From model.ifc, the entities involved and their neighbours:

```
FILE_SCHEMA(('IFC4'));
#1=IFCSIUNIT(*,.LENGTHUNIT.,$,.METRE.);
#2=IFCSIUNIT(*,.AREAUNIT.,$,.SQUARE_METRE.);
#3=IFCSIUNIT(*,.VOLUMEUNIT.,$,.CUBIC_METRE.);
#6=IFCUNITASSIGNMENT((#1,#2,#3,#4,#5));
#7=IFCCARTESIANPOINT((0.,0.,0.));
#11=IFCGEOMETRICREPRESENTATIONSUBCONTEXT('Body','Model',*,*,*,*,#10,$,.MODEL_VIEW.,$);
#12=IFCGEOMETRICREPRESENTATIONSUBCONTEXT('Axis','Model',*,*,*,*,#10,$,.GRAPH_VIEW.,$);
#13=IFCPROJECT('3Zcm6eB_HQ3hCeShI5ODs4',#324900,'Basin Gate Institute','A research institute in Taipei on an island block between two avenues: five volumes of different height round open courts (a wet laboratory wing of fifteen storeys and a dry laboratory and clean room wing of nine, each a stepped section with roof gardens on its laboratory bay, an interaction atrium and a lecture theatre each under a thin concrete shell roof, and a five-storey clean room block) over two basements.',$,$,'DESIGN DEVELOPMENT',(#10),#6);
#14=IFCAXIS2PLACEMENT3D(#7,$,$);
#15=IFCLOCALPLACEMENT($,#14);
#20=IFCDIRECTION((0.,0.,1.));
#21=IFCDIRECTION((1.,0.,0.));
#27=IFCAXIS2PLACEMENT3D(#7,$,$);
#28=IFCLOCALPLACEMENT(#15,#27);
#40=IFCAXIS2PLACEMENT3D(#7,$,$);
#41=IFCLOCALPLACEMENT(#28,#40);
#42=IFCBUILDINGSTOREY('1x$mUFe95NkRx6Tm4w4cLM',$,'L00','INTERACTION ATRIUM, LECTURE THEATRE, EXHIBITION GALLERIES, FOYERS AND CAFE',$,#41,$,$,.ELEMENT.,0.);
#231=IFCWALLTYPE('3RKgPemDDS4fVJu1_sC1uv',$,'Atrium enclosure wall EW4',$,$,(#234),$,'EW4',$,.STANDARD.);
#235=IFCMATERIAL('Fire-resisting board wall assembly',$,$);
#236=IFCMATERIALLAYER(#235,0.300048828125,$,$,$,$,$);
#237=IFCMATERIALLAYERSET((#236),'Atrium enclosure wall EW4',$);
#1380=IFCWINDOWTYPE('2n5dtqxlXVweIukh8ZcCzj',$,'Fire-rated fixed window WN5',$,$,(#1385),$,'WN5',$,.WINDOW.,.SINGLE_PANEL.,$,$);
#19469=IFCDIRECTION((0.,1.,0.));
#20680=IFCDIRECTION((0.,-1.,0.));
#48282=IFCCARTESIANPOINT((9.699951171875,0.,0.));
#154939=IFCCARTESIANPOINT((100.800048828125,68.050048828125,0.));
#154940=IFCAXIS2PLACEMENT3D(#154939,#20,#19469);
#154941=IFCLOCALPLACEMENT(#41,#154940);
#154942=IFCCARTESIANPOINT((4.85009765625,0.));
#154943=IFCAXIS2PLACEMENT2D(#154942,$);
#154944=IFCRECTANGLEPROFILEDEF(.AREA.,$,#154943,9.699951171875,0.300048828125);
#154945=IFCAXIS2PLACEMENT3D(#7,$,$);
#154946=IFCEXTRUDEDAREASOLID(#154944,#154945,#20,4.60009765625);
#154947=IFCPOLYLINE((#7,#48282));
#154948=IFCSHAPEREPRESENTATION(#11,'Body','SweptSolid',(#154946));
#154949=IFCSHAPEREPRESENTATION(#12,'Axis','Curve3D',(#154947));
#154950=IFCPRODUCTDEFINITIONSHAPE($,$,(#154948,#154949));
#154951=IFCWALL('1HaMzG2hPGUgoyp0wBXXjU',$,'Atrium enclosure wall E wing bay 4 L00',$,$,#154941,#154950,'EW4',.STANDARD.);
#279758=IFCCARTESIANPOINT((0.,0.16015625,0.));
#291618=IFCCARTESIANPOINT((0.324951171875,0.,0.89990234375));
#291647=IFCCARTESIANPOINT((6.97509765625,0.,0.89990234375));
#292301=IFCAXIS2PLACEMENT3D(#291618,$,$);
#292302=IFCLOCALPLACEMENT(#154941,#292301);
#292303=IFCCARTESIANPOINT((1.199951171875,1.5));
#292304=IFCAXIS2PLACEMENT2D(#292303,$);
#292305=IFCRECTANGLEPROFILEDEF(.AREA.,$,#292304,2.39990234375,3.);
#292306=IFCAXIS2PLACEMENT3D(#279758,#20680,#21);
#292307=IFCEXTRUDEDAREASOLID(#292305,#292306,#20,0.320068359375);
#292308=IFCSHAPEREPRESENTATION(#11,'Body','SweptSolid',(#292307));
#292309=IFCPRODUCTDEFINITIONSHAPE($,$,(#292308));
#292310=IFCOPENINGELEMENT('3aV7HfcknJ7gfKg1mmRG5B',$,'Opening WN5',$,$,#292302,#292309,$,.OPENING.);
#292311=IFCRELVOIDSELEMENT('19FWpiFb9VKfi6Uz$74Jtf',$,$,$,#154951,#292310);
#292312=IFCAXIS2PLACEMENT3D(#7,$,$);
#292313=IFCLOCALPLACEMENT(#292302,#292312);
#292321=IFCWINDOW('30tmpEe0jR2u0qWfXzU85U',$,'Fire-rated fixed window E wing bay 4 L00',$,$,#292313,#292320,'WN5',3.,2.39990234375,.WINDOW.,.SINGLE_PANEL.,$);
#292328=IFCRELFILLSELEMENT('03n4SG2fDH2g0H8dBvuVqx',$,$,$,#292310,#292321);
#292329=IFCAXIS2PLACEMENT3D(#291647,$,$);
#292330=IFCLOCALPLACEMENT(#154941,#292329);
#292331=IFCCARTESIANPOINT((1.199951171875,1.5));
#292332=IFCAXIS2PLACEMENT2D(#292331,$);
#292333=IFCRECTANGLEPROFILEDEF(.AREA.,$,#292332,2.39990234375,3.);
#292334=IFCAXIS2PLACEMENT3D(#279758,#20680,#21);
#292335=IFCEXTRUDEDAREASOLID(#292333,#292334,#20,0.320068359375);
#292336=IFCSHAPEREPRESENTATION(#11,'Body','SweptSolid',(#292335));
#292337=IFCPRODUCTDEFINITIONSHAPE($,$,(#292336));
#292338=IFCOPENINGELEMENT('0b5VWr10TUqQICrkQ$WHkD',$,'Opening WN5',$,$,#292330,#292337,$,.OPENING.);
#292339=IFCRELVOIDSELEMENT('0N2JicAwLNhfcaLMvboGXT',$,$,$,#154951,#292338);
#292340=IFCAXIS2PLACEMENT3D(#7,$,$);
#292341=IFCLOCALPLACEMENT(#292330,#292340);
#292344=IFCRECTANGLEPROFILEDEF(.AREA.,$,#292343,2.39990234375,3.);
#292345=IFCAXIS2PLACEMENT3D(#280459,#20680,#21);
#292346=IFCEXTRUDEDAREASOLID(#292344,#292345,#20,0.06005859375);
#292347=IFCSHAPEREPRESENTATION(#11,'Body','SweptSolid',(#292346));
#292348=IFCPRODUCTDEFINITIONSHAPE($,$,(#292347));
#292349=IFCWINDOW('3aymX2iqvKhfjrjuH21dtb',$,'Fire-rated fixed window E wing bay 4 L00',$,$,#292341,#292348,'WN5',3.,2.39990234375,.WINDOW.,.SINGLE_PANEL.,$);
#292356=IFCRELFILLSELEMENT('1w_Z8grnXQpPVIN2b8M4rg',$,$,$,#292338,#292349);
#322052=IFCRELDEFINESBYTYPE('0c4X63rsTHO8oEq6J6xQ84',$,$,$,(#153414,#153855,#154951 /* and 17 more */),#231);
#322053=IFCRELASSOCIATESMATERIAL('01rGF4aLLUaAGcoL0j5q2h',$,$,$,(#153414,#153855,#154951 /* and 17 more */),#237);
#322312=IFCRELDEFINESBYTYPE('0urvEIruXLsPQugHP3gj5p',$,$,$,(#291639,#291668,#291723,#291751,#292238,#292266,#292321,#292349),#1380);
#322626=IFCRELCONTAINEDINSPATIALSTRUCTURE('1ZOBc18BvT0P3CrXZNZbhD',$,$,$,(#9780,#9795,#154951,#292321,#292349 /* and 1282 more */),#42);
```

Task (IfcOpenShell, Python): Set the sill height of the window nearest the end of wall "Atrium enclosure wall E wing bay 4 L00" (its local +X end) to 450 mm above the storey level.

```python
import numpy as np
import ifcopenshell
import ifcopenshell.api.geometry
import ifcopenshell.geom
import ifcopenshell.util.element
import ifcopenshell.util.placement
import ifcopenshell.util.shape
import ifcopenshell.util.unit

model = ifcopenshell.open("model.ifc")
unit_scale = ifcopenshell.util.unit.calculate_unit_scale(model)

window = model.by_id(292349)
opening = window.FillsVoids[0].RelatingOpeningElement
storey = ifcopenshell.util.element.get_container(window, ifc_class="IfcBuildingStorey")
level = ifcopenshell.util.placement.get_local_placement(storey.ObjectPlacement)[2, 3]

# The opening's origin need not be at the sill, so measure its lowest point.
shape = ifcopenshell.geom.create_shape(ifcopenshell.geom.settings(), opening)
bottom = ifcopenshell.util.shape.get_shape_bottom_elevation(shape, shape.geometry) / unit_scale
dz = level + 0.45 / unit_scale - bottom

shift = np.array([0.0, 0.0, dz])
# The window is placed relative to its opening, so it follows when the opening moves.
matrix = ifcopenshell.util.placement.get_local_placement(opening.ObjectPlacement)
matrix[:3, 3] += shift
ifcopenshell.api.geometry.edit_object_placement(
    model, product=opening, matrix=matrix, is_si=False, should_transform_children=True
)

print(f"moved by {dz * unit_scale:+.3f} m")

model.write("model_rev.ifc")
```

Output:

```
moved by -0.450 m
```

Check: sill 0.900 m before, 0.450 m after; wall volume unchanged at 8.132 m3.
